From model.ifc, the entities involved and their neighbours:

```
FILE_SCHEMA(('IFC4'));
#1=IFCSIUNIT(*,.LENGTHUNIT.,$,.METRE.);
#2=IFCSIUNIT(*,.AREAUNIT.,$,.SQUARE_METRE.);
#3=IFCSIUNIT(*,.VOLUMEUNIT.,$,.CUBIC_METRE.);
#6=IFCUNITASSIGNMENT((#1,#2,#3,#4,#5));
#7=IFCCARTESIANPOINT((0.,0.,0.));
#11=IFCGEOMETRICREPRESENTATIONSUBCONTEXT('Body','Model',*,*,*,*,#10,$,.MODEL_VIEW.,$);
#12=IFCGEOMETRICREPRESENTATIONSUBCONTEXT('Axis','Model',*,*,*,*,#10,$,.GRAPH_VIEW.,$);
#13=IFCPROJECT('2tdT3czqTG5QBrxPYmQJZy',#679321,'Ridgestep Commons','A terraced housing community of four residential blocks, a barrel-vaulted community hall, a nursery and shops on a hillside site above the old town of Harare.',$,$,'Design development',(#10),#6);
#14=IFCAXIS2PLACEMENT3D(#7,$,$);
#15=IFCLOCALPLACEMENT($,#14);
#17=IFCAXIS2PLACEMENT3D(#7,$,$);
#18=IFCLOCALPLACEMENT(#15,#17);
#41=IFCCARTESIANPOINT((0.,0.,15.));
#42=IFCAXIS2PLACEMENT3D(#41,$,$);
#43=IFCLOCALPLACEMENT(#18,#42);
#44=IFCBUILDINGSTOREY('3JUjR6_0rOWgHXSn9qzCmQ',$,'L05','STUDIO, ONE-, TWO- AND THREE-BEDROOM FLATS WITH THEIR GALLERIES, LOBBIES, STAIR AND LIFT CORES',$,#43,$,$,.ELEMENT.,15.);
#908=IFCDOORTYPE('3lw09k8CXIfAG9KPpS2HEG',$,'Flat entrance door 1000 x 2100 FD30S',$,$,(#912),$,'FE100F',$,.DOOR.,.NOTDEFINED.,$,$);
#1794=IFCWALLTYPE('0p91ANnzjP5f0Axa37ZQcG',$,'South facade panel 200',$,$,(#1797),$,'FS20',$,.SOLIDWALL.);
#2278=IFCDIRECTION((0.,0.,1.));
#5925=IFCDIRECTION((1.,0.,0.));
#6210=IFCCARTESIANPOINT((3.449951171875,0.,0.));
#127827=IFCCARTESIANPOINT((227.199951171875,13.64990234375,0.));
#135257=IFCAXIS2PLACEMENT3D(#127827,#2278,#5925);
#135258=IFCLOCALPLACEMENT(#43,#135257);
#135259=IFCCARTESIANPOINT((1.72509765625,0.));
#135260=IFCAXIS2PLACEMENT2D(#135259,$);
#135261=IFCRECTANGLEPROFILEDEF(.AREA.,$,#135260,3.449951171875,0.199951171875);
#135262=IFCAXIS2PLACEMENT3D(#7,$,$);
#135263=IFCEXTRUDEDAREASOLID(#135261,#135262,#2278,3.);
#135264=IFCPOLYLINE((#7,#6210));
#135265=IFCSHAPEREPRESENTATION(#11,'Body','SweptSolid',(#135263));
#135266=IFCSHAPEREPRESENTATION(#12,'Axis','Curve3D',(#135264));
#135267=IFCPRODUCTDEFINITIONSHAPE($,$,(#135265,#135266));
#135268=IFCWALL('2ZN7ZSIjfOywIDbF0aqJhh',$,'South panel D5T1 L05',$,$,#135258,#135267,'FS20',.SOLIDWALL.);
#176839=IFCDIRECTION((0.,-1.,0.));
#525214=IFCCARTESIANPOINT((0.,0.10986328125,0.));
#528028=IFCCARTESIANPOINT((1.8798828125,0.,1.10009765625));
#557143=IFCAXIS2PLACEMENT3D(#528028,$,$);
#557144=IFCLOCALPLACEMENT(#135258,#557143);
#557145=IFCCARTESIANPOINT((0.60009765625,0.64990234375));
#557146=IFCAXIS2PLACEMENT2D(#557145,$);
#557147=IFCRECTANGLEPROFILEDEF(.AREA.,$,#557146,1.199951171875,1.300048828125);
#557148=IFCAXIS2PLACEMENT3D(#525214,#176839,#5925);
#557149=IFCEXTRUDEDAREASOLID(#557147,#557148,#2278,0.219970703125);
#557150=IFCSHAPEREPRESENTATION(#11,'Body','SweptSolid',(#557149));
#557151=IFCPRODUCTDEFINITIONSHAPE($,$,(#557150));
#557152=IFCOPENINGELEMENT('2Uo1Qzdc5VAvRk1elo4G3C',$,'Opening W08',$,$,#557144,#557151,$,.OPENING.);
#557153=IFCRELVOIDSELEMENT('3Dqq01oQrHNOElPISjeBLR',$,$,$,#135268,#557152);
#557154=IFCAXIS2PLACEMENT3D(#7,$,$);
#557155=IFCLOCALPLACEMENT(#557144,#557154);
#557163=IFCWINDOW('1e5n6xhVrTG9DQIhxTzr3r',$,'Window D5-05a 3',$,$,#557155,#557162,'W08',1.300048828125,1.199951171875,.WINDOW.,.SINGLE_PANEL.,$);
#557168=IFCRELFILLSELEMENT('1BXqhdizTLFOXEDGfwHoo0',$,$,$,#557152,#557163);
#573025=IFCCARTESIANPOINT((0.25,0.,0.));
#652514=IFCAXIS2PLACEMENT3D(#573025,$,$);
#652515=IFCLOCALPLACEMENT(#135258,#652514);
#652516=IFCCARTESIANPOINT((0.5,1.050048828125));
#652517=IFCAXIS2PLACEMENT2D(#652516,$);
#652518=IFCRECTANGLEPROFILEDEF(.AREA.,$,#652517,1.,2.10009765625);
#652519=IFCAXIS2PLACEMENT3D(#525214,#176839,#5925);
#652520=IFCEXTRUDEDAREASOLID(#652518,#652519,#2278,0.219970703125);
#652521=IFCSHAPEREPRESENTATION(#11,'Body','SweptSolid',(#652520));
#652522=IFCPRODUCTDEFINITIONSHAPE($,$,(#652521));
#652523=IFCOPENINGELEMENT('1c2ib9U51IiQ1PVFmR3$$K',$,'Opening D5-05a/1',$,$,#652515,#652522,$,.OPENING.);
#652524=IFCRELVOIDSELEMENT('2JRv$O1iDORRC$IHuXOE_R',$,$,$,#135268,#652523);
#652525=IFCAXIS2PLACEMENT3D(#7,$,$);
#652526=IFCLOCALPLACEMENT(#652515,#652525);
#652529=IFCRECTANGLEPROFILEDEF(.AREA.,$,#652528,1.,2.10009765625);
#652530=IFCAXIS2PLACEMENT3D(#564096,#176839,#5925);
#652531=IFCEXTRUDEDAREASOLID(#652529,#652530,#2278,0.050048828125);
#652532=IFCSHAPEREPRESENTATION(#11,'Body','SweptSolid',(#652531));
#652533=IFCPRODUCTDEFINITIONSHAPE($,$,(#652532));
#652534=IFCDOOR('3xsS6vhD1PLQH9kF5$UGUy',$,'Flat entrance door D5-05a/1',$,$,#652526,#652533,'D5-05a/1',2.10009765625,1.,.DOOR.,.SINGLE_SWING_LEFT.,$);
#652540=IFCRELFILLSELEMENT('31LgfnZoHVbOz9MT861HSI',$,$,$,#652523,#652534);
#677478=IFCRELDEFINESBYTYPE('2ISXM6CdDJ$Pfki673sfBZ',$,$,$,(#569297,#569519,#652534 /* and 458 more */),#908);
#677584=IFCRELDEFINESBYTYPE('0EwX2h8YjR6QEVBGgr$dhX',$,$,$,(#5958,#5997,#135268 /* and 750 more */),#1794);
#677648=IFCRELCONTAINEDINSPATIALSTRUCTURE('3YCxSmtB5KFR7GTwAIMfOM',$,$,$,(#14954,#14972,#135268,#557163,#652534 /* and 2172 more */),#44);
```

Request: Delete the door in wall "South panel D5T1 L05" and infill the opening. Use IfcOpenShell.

```python
import ifcopenshell
import ifcopenshell.api.feature
import ifcopenshell.api.root
import ifcopenshell.geom
import ifcopenshell.util.shape

model = ifcopenshell.open("model.ifc")
settings = ifcopenshell.geom.settings()


def volume(element):
    """Net volume in cubic metres, openings subtracted."""
    shape = ifcopenshell.geom.create_shape(settings, element)
    return ifcopenshell.util.shape.get_volume(shape.geometry)


door = model.by_guid("3xsS6vhD1PLQH9kF5$UGUy")
opening = door.FillsVoids[0].RelatingOpeningElement
wall = opening.VoidsElements[0].RelatingBuildingElement
before = volume(wall)

ifcopenshell.api.root.remove_product(model, product=door)
ifcopenshell.api.feature.remove_feature(model, feature=opening)

after = volume(wall)

print(f"wall volume {before:.3f} -> {after:.3f} m3")

model.write("model-out.ifc")
```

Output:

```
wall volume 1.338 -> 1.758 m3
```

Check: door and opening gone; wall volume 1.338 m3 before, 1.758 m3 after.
